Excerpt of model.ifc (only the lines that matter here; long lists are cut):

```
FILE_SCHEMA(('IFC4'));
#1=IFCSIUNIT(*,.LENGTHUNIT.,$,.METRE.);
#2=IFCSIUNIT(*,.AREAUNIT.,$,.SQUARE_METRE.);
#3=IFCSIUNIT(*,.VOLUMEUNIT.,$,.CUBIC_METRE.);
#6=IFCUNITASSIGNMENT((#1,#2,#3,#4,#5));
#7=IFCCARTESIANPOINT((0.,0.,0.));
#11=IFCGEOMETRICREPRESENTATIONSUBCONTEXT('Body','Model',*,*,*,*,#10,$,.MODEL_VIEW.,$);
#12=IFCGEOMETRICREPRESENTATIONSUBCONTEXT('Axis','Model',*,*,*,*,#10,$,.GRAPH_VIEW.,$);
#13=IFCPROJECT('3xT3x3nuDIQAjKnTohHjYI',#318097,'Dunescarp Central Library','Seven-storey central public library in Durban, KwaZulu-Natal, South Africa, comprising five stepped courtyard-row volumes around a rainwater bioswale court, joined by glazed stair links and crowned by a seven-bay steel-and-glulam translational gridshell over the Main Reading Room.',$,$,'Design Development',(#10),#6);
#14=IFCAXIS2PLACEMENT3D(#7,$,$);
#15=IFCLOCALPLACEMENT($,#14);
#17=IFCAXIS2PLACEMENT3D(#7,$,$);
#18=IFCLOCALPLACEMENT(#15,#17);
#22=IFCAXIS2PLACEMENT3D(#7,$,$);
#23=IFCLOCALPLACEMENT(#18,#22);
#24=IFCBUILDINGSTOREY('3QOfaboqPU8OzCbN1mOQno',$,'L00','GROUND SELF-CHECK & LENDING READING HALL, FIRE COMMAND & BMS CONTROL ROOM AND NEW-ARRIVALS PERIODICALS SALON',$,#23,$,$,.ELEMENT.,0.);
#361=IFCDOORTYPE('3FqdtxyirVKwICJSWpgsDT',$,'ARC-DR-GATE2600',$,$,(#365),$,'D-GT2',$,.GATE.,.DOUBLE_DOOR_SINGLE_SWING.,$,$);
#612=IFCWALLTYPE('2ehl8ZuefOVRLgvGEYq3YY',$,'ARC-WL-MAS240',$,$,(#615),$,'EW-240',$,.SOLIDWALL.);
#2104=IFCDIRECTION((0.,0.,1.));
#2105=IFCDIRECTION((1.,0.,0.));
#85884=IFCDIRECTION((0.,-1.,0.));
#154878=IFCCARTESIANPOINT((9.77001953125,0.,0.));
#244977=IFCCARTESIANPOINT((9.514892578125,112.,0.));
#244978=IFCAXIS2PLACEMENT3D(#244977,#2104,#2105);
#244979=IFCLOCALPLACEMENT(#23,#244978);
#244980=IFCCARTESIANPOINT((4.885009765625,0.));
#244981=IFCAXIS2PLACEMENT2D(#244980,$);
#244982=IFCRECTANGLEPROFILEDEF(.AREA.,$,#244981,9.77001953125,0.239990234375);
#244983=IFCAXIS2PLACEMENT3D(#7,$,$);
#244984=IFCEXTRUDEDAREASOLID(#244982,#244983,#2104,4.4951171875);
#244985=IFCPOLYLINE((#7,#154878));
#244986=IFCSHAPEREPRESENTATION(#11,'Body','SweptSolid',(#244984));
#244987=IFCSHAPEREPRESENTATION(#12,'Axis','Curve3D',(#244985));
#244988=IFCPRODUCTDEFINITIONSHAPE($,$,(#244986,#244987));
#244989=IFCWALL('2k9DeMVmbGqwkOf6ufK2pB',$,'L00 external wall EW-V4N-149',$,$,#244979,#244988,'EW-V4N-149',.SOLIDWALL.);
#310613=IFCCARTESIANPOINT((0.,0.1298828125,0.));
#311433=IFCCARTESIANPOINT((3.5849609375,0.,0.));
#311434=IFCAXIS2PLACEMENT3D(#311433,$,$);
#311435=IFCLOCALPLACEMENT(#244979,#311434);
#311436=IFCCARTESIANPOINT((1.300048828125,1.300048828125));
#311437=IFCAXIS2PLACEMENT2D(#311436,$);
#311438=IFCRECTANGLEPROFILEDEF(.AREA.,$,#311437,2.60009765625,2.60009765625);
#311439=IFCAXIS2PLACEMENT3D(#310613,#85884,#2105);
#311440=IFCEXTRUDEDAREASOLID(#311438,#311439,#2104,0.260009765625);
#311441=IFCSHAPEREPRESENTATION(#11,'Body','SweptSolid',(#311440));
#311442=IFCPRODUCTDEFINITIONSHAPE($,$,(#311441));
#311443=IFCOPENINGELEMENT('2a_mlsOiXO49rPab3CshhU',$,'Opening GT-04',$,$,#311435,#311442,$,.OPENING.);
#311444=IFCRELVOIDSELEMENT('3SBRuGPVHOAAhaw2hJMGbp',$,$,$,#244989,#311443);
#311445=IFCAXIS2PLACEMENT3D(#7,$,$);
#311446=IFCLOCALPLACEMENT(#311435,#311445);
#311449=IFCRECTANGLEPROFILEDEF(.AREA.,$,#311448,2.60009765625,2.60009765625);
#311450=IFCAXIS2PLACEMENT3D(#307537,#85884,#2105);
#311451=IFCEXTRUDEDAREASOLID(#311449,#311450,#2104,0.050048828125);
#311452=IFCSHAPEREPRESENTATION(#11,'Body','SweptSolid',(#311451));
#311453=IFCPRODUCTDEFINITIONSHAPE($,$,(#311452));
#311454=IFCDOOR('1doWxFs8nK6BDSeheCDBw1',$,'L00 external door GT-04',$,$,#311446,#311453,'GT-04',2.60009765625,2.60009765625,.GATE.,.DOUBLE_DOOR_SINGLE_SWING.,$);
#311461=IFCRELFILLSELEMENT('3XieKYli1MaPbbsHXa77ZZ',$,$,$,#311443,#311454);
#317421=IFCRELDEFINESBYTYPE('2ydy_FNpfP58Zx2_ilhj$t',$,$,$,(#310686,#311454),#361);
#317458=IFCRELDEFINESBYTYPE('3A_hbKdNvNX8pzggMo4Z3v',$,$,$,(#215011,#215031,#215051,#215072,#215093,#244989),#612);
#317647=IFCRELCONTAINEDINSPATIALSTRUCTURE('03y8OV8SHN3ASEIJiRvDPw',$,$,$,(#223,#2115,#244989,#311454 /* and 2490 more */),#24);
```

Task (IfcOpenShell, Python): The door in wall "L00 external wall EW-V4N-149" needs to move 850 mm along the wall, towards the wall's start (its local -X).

```python
import ifcopenshell
import ifcopenshell.api.geometry
import ifcopenshell.util.placement
import ifcopenshell.util.unit

model = ifcopenshell.open("model.ifc")
unit_scale = ifcopenshell.util.unit.calculate_unit_scale(model)

door = model.by_id(311454)
opening = door.FillsVoids[0].RelatingOpeningElement
wall = opening.VoidsElements[0].RelatingBuildingElement

wall_matrix = ifcopenshell.util.placement.get_local_placement(wall.ObjectPlacement)
shift = wall_matrix[:3, 0] * -0.85 / unit_scale
before = ifcopenshell.util.placement.get_local_placement(door.ObjectPlacement)[:3, 3].copy()

# The door is placed relative to its opening, so it follows when the opening moves.
matrix = ifcopenshell.util.placement.get_local_placement(opening.ObjectPlacement)
matrix[:3, 3] += shift
ifcopenshell.api.geometry.edit_object_placement(
    model, product=opening, matrix=matrix, is_si=False, should_transform_children=True
)

after = ifcopenshell.util.placement.get_local_placement(door.ObjectPlacement)[:3, 3]
print("door moved by", (after - before).round(3) + 0.0)

model.write("model-out.ifc")
```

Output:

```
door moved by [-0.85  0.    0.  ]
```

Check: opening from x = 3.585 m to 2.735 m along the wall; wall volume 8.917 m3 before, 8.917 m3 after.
